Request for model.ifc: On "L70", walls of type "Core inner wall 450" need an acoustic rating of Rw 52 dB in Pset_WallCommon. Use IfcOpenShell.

First a look at what the model holds.

```python
import ifcopenshell
import ifcopenshell.util.element

model = ifcopenshell.open("model.ifc")
print(model.schema)
storey = next(s for s in model.by_type("IfcBuildingStorey") if s.Name == "L70")
walls = [e for e in ifcopenshell.util.element.get_decomposition(storey) if e.is_a("IfcWall")]
seen = {}
for e in walls:
    element_type = ifcopenshell.util.element.get_type(e)
    key = (element_type.Name if element_type != e and element_type else None, ifcopenshell.util.element.get_pset(e, "Pset_WallCommon", "AcousticRating"))
    seen[key] = seen.get(key, 0) + 1
for (name, value), count in sorted(seen.items(), key=str):
    print(count, "x", name, "|", value)
```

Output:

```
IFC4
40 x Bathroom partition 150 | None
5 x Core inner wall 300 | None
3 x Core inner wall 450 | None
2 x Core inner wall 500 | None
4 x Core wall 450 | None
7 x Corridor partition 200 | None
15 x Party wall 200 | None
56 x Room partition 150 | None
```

```python
import ifcopenshell
import ifcopenshell.api.pset
import ifcopenshell.util.element

model = ifcopenshell.open("model.ifc")

storey = next(s for s in model.by_type("IfcBuildingStorey") if s.Name == "L70")
walls = [e for e in ifcopenshell.util.element.get_decomposition(storey) if e.is_a("IfcWall")]

count = 0
for e in walls:
    element_type = ifcopenshell.util.element.get_type(e)
    if element_type in (None, e) or element_type.Name != "Core inner wall 450":
        continue
    found = ifcopenshell.util.element.get_pset(e, "Pset_WallCommon", should_inherit=False)
    if found:
        pset = model.by_id(found["id"])
        if len(ifcopenshell.util.element.get_elements_by_pset(pset)) > 1:
            pset = ifcopenshell.api.pset.unshare_pset(model, products=[e], pset=pset)[0]
    else:
        pset = ifcopenshell.api.pset.add_pset(model, product=e, name="Pset_WallCommon")
    ifcopenshell.api.pset.edit_pset(model, pset=pset, properties={"AcousticRating": "Rw 52 dB"})
    count += 1

print(count, "walls updated")

model.write("model_v2.ifc")
```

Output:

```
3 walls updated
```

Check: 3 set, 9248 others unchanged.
